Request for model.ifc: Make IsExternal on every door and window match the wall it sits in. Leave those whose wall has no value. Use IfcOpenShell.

First a look at what the model holds.

```python
import ifcopenshell
import ifcopenshell.util.element

model = ifcopenshell.open("model.ifc")
print(model.schema)
seen = {}
for e in model.by_type("IfcDoor") + model.by_type("IfcWindow"):
    if not e.FillsVoids:
        continue
    host = e.FillsVoids[0].RelatingOpeningElement.VoidsElements[0].RelatingBuildingElement
    own = ifcopenshell.util.element.get_pset(e, f"Pset_{e.is_a()[3:].removesuffix('StandardCase')}Common", "IsExternal")
    wall = ifcopenshell.util.element.get_pset(host, "Pset_WallCommon", "IsExternal")
    seen[e.is_a(), own, wall] = seen.get((e.is_a(), own, wall), 0) + 1
for (cls, own, wall), count in sorted(seen.items(), key=str):
    print(count, cls, "IsExternal:", own, "| host wall:", wall)
```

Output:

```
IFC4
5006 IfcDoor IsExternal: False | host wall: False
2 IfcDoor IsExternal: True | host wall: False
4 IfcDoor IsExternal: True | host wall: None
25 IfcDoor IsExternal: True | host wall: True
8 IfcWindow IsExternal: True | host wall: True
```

```python
import ifcopenshell
import ifcopenshell.api.pset
import ifcopenshell.util.element

model = ifcopenshell.open("model.ifc")

count = 0
for ifc_class, pset_name in (("IfcDoor", "Pset_DoorCommon"), ("IfcWindow", "Pset_WindowCommon")):
    for e in model.by_type(ifc_class):
        if not e.FillsVoids:
            continue
        host = e.FillsVoids[0].RelatingOpeningElement.VoidsElements[0].RelatingBuildingElement
        external = ifcopenshell.util.element.get_pset(host, "Pset_WallCommon", "IsExternal")
        if external is None or ifcopenshell.util.element.get_pset(e, pset_name, "IsExternal") == external:
            continue
        pset = ifcopenshell.api.pset.add_pset(model, product=e, name=pset_name)
        ifcopenshell.api.pset.edit_pset(model, pset=pset, properties={"IsExternal": external})
        count += 1

print(count, "updated")

model.write("model_v2.ifc")
```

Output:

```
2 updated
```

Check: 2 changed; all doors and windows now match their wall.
